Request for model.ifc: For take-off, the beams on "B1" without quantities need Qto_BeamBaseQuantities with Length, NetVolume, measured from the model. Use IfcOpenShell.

First a look at what the model holds.

```python
import ifcopenshell
import ifcopenshell.util.element
import ifcopenshell.util.unit

model = ifcopenshell.open("model.ifc")
print(model.schema)
for unit_type in ("LENGTHUNIT", "AREAUNIT", "VOLUMEUNIT"):
    print(unit_type, ifcopenshell.util.unit.calculate_unit_scale(model, unit_type))
storey = next(s for s in model.by_type("IfcBuildingStorey") if s.Name == "B1")
beams = [e for e in ifcopenshell.util.element.get_decomposition(storey) if e.is_a("IfcBeam")]
for e in sorted(beams, key=lambda e: e.id()):
    print(e.id(), e.is_a(), e.Name, list(ifcopenshell.util.element.get_psets(e, qtos_only=True)), sep=" | ")
```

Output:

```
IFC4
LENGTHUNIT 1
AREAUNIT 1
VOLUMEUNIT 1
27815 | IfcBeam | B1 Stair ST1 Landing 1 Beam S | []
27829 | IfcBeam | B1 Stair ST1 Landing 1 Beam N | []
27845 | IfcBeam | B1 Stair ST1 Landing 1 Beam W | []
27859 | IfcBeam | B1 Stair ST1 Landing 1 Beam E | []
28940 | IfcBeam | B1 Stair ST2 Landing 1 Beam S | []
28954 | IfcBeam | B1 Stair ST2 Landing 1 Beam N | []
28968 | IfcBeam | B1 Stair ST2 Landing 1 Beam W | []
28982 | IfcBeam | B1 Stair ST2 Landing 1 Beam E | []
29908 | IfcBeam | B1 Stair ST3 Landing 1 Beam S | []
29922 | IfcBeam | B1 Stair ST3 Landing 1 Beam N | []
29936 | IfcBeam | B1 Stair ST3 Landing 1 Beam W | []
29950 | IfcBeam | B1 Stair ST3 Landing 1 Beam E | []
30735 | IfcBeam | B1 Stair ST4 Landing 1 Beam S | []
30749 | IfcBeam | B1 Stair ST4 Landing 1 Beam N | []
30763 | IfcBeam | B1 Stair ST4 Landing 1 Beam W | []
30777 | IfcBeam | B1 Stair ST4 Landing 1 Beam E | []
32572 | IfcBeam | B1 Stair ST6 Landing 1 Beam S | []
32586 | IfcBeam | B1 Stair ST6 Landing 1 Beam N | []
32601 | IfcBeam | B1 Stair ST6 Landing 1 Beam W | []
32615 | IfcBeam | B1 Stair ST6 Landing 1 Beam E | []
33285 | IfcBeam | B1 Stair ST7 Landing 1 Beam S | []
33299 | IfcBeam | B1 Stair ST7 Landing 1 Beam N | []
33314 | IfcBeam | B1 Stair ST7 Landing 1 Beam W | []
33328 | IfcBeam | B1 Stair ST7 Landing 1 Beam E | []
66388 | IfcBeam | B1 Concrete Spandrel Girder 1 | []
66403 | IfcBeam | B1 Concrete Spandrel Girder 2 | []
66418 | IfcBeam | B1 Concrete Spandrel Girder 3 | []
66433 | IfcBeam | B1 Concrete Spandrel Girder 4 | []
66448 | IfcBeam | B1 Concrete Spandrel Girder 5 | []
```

```python
import ifcopenshell
import ifcopenshell.api.pset
import ifcopenshell.geom
import ifcopenshell.util.element
import ifcopenshell.util.shape
import ifcopenshell.util.unit

model = ifcopenshell.open("model.ifc")
unit_scale = ifcopenshell.util.unit.calculate_unit_scale(model)
volume_scale = ifcopenshell.util.unit.calculate_unit_scale(model, "VOLUMEUNIT")
settings = ifcopenshell.geom.settings()

storey = next(s for s in model.by_type("IfcBuildingStorey") if s.Name == "B1")
beams = [e for e in ifcopenshell.util.element.get_decomposition(storey) if e.is_a("IfcBeam")]

for e in sorted(beams, key=lambda e: e.id()):
    if ifcopenshell.util.element.get_psets(e, qtos_only=True, should_inherit=False):
        continue
    # Geometry comes back in metres, in the element's own axes.
    shape = ifcopenshell.geom.create_shape(settings, e)
    values = {
        "Length": ifcopenshell.util.shape.get_max_xyz(shape.geometry) / unit_scale,
        "NetVolume": ifcopenshell.util.shape.get_volume(shape.geometry) / volume_scale,
    }
    qto = ifcopenshell.api.pset.add_qto(model, product=e, name="Qto_BeamBaseQuantities")
    ifcopenshell.api.pset.edit_qto(model, qto=qto, properties=values)
    print(e.id(), {k: round(v, 3) for k, v in values.items()})

model.write("model_updated.ifc")
```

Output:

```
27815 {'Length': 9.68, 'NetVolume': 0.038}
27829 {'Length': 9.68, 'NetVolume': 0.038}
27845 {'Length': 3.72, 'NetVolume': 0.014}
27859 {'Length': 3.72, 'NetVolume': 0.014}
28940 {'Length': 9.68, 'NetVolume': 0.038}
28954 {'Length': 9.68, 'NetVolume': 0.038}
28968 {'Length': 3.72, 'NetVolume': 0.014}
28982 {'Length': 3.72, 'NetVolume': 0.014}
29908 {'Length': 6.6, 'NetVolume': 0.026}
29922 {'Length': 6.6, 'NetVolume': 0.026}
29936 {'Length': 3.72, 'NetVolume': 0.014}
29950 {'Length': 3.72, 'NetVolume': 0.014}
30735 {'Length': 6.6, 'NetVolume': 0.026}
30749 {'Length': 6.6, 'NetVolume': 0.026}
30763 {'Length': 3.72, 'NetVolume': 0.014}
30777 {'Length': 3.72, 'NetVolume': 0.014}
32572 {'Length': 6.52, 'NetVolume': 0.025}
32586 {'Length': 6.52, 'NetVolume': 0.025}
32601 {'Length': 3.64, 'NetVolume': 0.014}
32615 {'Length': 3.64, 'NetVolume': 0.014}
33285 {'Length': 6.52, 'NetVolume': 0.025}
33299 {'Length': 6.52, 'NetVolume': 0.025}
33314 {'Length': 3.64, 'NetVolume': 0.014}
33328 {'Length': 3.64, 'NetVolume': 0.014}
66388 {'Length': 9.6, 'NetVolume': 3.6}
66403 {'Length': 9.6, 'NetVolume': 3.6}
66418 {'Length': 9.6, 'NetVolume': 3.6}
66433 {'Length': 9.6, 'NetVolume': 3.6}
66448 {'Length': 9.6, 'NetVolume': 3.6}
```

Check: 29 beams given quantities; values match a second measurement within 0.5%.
